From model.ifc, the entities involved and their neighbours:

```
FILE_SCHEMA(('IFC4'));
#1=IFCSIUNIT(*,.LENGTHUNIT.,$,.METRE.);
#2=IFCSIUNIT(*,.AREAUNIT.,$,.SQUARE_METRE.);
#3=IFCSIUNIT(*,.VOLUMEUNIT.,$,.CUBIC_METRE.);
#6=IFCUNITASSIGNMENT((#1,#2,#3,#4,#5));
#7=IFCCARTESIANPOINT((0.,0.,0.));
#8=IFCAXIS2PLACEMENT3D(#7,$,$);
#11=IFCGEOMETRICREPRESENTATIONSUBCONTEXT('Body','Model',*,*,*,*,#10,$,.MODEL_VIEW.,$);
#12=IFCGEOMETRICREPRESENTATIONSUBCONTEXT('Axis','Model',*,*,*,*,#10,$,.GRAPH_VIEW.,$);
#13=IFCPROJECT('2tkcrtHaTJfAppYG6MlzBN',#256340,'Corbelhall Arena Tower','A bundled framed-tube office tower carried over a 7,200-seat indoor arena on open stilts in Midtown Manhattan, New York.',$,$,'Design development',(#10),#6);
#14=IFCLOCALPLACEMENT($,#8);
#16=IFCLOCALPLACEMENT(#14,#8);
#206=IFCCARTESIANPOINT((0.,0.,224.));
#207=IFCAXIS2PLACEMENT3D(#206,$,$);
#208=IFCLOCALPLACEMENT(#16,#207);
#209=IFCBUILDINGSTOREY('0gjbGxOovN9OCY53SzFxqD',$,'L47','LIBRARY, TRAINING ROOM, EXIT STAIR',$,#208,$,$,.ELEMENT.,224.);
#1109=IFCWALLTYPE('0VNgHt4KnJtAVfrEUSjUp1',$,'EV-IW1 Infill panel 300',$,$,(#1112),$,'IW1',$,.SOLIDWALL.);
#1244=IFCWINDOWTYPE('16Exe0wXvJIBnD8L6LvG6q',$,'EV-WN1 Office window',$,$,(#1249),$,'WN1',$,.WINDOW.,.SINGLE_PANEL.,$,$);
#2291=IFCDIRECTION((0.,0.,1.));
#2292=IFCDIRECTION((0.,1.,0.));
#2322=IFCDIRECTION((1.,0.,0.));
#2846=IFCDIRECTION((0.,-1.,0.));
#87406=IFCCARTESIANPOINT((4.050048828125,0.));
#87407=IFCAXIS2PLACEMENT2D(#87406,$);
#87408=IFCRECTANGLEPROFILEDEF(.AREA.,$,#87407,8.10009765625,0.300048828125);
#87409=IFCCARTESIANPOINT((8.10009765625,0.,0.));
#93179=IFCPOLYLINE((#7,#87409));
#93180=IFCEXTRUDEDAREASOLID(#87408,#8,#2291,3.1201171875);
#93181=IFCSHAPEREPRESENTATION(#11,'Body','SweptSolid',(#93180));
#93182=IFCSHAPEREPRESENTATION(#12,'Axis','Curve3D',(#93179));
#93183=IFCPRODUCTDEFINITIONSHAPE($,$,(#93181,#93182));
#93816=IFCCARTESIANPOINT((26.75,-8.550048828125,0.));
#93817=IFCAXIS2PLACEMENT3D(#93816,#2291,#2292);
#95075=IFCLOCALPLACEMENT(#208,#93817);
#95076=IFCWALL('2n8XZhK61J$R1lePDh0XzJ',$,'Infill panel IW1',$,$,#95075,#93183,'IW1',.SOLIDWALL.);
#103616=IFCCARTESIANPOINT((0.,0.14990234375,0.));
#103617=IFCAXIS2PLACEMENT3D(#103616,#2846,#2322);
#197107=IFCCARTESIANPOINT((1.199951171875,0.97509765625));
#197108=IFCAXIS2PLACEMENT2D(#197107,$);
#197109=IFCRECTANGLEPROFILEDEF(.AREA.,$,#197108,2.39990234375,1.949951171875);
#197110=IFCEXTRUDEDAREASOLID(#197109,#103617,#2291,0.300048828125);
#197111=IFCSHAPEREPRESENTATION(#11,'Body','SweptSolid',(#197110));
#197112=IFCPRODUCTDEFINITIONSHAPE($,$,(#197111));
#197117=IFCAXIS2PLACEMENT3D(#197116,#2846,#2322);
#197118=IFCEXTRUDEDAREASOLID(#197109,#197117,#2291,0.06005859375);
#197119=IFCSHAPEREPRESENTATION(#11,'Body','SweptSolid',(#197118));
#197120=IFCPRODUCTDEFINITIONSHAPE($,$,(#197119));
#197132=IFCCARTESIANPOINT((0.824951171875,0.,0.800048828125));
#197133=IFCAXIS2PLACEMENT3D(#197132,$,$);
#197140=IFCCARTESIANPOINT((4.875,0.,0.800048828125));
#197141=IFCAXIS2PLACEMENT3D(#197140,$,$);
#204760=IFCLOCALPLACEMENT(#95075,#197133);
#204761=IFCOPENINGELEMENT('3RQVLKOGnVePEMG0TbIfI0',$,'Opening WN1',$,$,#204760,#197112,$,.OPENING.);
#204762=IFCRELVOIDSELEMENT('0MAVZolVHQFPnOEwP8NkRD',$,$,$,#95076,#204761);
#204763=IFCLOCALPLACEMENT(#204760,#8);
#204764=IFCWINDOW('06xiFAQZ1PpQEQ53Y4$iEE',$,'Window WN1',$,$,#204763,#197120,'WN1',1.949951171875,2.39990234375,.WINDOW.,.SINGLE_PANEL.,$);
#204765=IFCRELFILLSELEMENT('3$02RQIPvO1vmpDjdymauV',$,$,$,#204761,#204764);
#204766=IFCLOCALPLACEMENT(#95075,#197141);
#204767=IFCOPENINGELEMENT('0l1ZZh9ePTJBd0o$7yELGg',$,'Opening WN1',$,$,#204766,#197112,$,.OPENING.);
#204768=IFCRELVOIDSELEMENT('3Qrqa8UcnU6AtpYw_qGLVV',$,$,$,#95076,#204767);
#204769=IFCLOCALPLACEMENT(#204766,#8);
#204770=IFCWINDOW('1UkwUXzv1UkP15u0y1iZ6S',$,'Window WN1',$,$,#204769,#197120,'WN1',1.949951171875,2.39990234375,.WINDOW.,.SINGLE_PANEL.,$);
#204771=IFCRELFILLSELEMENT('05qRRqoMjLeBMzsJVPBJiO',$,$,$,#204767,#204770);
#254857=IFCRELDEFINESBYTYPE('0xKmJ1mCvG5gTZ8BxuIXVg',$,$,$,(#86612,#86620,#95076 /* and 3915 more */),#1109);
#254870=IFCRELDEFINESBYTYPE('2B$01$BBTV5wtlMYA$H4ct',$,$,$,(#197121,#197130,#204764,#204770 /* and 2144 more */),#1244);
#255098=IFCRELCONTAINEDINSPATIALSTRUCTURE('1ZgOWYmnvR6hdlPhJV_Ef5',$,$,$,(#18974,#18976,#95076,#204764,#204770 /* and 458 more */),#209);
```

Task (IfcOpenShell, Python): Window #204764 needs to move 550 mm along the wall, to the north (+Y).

```python
import ifcopenshell
import ifcopenshell.api.geometry
import ifcopenshell.util.placement
import ifcopenshell.util.unit

model = ifcopenshell.open("model.ifc")
unit_scale = ifcopenshell.util.unit.calculate_unit_scale(model)

window = model.by_id(204764)
opening = window.FillsVoids[0].RelatingOpeningElement
wall = opening.VoidsElements[0].RelatingBuildingElement

wall_matrix = ifcopenshell.util.placement.get_local_placement(wall.ObjectPlacement)
shift = wall_matrix[:3, 0] * 0.55 / unit_scale
before = ifcopenshell.util.placement.get_local_placement(window.ObjectPlacement)[:3, 3].copy()

# The window is placed relative to its opening, so it follows when the opening moves.
matrix = ifcopenshell.util.placement.get_local_placement(opening.ObjectPlacement)
matrix[:3, 3] += shift
ifcopenshell.api.geometry.edit_object_placement(
    model, product=opening, matrix=matrix, is_si=False, should_transform_children=True
)

after = ifcopenshell.util.placement.get_local_placement(window.ObjectPlacement)[:3, 3]
print("window moved by", (after - before).round(3) + 0.0)

model.write("model_updated.ifc")
```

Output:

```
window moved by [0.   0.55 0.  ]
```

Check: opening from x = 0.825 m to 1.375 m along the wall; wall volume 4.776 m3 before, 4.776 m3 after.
